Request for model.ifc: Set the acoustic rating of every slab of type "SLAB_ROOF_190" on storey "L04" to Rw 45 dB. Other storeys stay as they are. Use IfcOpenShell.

First a look at what the model holds.

```python
import ifcopenshell
import ifcopenshell.util.element

model = ifcopenshell.open("model.ifc")
print(model.schema)
storey = next(s for s in model.by_type("IfcBuildingStorey") if s.Name == "L04")
slabs = [e for e in ifcopenshell.util.element.get_decomposition(storey) if e.is_a("IfcSlab")]
seen = {}
for e in slabs:
    element_type = ifcopenshell.util.element.get_type(e)
    key = (element_type.Name if element_type != e and element_type else None, ifcopenshell.util.element.get_pset(e, "Pset_SlabCommon", "AcousticRating"))
    seen[key] = seen.get(key, 0) + 1
for (name, value), count in sorted(seen.items(), key=str):
    print(count, "x", name, "|", value)
```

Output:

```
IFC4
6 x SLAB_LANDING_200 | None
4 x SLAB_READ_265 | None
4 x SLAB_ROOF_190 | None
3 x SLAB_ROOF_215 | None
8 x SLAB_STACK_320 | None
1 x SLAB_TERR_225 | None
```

```python
import ifcopenshell
import ifcopenshell.api.pset
import ifcopenshell.util.element

model = ifcopenshell.open("model.ifc")

storey = next(s for s in model.by_type("IfcBuildingStorey") if s.Name == "L04")
slabs = [e for e in ifcopenshell.util.element.get_decomposition(storey) if e.is_a("IfcSlab")]

count = 0
for e in slabs:
    element_type = ifcopenshell.util.element.get_type(e)
    if element_type in (None, e) or element_type.Name != "SLAB_ROOF_190":
        continue
    # add_pset returns the element's existing set when there is one.
    pset = ifcopenshell.api.pset.add_pset(model, product=e, name="Pset_SlabCommon")
    ifcopenshell.api.pset.edit_pset(model, pset=pset, properties={"AcousticRating": "Rw 45 dB"})
    count += 1

print(count, "slabs updated")

model.write("model_v2.ifc")
```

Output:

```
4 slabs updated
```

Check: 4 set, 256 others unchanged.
